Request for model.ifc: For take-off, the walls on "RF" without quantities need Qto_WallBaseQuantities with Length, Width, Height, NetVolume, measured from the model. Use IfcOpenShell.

First a look at what the model holds.

```python
import ifcopenshell
import ifcopenshell.util.element
import ifcopenshell.util.unit

model = ifcopenshell.open("model.ifc")
print(model.schema)
for unit_type in ("LENGTHUNIT", "AREAUNIT", "VOLUMEUNIT"):
    print(unit_type, ifcopenshell.util.unit.calculate_unit_scale(model, unit_type))
storey = next(s for s in model.by_type("IfcBuildingStorey") if s.Name == "RF")
walls = [e for e in ifcopenshell.util.element.get_decomposition(storey) if e.is_a("IfcWall")]
for e in sorted(walls, key=lambda e: e.id()):
    print(e.id(), e.is_a(), e.Name, list(ifcopenshell.util.element.get_psets(e, qtos_only=True)), sep=" | ")
```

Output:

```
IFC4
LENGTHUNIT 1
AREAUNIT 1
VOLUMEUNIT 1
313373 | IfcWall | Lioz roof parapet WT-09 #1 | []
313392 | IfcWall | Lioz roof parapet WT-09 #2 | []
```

```python
import ifcopenshell
import ifcopenshell.api.pset
import ifcopenshell.geom
import ifcopenshell.util.element
import ifcopenshell.util.shape
import ifcopenshell.util.unit

model = ifcopenshell.open("model.ifc")
unit_scale = ifcopenshell.util.unit.calculate_unit_scale(model)
volume_scale = ifcopenshell.util.unit.calculate_unit_scale(model, "VOLUMEUNIT")
settings = ifcopenshell.geom.settings()

storey = next(s for s in model.by_type("IfcBuildingStorey") if s.Name == "RF")
walls = [e for e in ifcopenshell.util.element.get_decomposition(storey) if e.is_a("IfcWall")]

for e in sorted(walls, key=lambda e: e.id()):
    if ifcopenshell.util.element.get_psets(e, qtos_only=True, should_inherit=False):
        continue
    # Geometry comes back in metres, in the element's own axes.
    shape = ifcopenshell.geom.create_shape(settings, e)
    values = {
        "Length": ifcopenshell.util.shape.get_x(shape.geometry) / unit_scale,
        "Width": ifcopenshell.util.shape.get_y(shape.geometry) / unit_scale,
        "Height": ifcopenshell.util.shape.get_z(shape.geometry) / unit_scale,
        "NetVolume": ifcopenshell.util.shape.get_volume(shape.geometry) / volume_scale,
    }
    qto = ifcopenshell.api.pset.add_qto(model, product=e, name="Qto_WallBaseQuantities")
    ifcopenshell.api.pset.edit_qto(model, qto=qto, properties=values)
    print(e.id(), {k: round(v, 3) for k, v in values.items()})

model.write("model_rev.ifc")
```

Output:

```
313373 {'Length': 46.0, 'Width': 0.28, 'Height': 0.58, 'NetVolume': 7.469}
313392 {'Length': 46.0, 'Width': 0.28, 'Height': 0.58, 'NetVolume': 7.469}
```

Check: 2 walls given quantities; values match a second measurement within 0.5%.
